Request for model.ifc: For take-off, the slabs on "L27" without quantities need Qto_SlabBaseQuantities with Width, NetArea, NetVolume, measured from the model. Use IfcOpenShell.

First a look at what the model holds.

```python
import ifcopenshell
import ifcopenshell.util.element
import ifcopenshell.util.unit

model = ifcopenshell.open("model.ifc")
print(model.schema)
for unit_type in ("LENGTHUNIT", "AREAUNIT", "VOLUMEUNIT"):
    print(unit_type, ifcopenshell.util.unit.calculate_unit_scale(model, unit_type))
storey = next(s for s in model.by_type("IfcBuildingStorey") if s.Name == "L27")
slabs = [e for e in ifcopenshell.util.element.get_decomposition(storey) if e.is_a("IfcSlab")]
for e in sorted(slabs, key=lambda e: e.id()):
    print(e.id(), e.is_a(), e.Name, list(ifcopenshell.util.element.get_psets(e, qtos_only=True)), sep=" | ")
```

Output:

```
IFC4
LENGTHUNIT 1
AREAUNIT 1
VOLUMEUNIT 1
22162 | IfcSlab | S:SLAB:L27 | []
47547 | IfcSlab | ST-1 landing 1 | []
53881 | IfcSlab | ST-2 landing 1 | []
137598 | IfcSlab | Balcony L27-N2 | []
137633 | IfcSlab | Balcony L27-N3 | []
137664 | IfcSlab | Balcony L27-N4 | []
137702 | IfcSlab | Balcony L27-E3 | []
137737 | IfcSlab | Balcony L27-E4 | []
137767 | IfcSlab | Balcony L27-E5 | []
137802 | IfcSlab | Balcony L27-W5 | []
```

```python
import ifcopenshell
import ifcopenshell.api.pset
import ifcopenshell.geom
import ifcopenshell.util.element
import ifcopenshell.util.shape
import ifcopenshell.util.unit

model = ifcopenshell.open("model.ifc")
unit_scale = ifcopenshell.util.unit.calculate_unit_scale(model)
area_scale = ifcopenshell.util.unit.calculate_unit_scale(model, "AREAUNIT")
volume_scale = ifcopenshell.util.unit.calculate_unit_scale(model, "VOLUMEUNIT")
settings = ifcopenshell.geom.settings()

storey = next(s for s in model.by_type("IfcBuildingStorey") if s.Name == "L27")
slabs = [e for e in ifcopenshell.util.element.get_decomposition(storey) if e.is_a("IfcSlab")]

for e in sorted(slabs, key=lambda e: e.id()):
    if ifcopenshell.util.element.get_psets(e, qtos_only=True, should_inherit=False):
        continue
    # Geometry comes back in metres, in the element's own axes.
    shape = ifcopenshell.geom.create_shape(settings, e)
    values = {
        "Width": ifcopenshell.util.shape.get_z(shape.geometry) / unit_scale,
        "NetArea": ifcopenshell.util.shape.get_footprint_area(shape.geometry) / area_scale,
        "NetVolume": ifcopenshell.util.shape.get_volume(shape.geometry) / volume_scale,
    }
    qto = ifcopenshell.api.pset.add_qto(model, product=e, name="Qto_SlabBaseQuantities")
    ifcopenshell.api.pset.edit_qto(model, qto=qto, properties=values)
    print(e.id(), {k: round(v, 3) for k, v in values.items()})

model.write("model_v2.ifc")
```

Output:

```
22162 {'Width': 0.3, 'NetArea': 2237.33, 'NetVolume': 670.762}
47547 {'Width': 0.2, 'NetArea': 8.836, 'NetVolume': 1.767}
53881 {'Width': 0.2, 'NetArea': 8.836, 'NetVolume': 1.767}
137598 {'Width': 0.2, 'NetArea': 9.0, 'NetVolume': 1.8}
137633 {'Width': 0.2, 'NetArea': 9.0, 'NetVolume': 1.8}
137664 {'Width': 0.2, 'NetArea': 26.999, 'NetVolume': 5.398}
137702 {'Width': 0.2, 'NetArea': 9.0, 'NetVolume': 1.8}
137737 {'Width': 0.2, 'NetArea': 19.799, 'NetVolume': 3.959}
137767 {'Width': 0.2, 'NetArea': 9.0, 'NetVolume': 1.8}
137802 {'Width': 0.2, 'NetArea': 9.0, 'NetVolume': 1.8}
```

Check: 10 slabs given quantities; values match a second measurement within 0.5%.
